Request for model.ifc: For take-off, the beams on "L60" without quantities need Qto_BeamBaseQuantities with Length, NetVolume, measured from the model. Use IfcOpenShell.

First a look at what the model holds.

```python
import ifcopenshell
import ifcopenshell.util.element
import ifcopenshell.util.unit

model = ifcopenshell.open("model.ifc")
print(model.schema)
for unit_type in ("LENGTHUNIT", "AREAUNIT", "VOLUMEUNIT"):
    print(unit_type, ifcopenshell.util.unit.calculate_unit_scale(model, unit_type))
storey = next(s for s in model.by_type("IfcBuildingStorey") if s.Name == "L60")
beams = [e for e in ifcopenshell.util.element.get_decomposition(storey) if e.is_a("IfcBeam")]
for e in sorted(beams, key=lambda e: e.id()):
    print(e.id(), e.is_a(), e.Name, list(ifcopenshell.util.element.get_psets(e, qtos_only=True)), sep=" | ")
```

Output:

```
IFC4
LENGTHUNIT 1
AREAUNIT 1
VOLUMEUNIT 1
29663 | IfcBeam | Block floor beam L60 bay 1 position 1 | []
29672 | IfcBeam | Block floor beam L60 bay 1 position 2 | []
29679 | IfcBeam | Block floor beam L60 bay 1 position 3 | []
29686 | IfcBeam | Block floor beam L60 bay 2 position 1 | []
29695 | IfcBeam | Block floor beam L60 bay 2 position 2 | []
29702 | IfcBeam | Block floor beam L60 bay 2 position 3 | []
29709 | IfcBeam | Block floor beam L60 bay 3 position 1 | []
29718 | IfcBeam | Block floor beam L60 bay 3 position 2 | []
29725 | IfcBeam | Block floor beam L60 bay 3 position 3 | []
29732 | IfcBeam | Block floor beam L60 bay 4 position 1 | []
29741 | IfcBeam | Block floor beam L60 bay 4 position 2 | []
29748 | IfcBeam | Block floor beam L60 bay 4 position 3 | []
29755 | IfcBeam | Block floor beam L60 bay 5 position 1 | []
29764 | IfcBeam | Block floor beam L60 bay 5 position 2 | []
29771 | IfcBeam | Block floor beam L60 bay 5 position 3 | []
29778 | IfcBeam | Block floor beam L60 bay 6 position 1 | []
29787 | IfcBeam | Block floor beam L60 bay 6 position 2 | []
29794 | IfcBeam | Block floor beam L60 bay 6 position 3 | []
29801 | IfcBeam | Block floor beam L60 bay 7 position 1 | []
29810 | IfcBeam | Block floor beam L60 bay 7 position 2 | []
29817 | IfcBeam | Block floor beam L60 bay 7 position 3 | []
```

```python
import ifcopenshell
import ifcopenshell.api.pset
import ifcopenshell.geom
import ifcopenshell.util.element
import ifcopenshell.util.shape
import ifcopenshell.util.unit

model = ifcopenshell.open("model.ifc")
unit_scale = ifcopenshell.util.unit.calculate_unit_scale(model)
volume_scale = ifcopenshell.util.unit.calculate_unit_scale(model, "VOLUMEUNIT")
settings = ifcopenshell.geom.settings()

storey = next(s for s in model.by_type("IfcBuildingStorey") if s.Name == "L60")
beams = [e for e in ifcopenshell.util.element.get_decomposition(storey) if e.is_a("IfcBeam")]

for e in sorted(beams, key=lambda e: e.id()):
    if ifcopenshell.util.element.get_psets(e, qtos_only=True, should_inherit=False):
        continue
    # Geometry comes back in metres, in the element's own axes.
    shape = ifcopenshell.geom.create_shape(settings, e)
    values = {
        "Length": ifcopenshell.util.shape.get_max_xyz(shape.geometry) / unit_scale,
        "NetVolume": ifcopenshell.util.shape.get_volume(shape.geometry) / volume_scale,
    }
    qto = ifcopenshell.api.pset.add_qto(model, product=e, name="Qto_BeamBaseQuantities")
    ifcopenshell.api.pset.edit_qto(model, qto=qto, properties=values)
    print(e.id(), {k: round(v, 3) for k, v in values.items()})

model.write("model_v2.ifc")
```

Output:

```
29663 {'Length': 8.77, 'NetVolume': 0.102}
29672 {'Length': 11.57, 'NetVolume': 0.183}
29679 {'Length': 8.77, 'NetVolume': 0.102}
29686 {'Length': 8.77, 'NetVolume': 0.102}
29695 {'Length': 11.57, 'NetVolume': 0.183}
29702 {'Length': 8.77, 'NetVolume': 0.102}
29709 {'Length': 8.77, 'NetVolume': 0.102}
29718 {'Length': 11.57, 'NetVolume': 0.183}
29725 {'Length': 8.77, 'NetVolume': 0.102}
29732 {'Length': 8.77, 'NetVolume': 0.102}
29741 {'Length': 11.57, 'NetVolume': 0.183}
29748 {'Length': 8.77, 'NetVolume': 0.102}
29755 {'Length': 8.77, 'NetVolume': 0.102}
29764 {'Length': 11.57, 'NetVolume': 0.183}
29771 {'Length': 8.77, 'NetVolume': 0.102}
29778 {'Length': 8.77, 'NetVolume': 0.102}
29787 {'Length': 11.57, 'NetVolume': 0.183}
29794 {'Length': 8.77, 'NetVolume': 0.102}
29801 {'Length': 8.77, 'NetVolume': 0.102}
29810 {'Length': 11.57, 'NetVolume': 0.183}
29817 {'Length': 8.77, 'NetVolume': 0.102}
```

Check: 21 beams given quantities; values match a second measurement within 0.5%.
